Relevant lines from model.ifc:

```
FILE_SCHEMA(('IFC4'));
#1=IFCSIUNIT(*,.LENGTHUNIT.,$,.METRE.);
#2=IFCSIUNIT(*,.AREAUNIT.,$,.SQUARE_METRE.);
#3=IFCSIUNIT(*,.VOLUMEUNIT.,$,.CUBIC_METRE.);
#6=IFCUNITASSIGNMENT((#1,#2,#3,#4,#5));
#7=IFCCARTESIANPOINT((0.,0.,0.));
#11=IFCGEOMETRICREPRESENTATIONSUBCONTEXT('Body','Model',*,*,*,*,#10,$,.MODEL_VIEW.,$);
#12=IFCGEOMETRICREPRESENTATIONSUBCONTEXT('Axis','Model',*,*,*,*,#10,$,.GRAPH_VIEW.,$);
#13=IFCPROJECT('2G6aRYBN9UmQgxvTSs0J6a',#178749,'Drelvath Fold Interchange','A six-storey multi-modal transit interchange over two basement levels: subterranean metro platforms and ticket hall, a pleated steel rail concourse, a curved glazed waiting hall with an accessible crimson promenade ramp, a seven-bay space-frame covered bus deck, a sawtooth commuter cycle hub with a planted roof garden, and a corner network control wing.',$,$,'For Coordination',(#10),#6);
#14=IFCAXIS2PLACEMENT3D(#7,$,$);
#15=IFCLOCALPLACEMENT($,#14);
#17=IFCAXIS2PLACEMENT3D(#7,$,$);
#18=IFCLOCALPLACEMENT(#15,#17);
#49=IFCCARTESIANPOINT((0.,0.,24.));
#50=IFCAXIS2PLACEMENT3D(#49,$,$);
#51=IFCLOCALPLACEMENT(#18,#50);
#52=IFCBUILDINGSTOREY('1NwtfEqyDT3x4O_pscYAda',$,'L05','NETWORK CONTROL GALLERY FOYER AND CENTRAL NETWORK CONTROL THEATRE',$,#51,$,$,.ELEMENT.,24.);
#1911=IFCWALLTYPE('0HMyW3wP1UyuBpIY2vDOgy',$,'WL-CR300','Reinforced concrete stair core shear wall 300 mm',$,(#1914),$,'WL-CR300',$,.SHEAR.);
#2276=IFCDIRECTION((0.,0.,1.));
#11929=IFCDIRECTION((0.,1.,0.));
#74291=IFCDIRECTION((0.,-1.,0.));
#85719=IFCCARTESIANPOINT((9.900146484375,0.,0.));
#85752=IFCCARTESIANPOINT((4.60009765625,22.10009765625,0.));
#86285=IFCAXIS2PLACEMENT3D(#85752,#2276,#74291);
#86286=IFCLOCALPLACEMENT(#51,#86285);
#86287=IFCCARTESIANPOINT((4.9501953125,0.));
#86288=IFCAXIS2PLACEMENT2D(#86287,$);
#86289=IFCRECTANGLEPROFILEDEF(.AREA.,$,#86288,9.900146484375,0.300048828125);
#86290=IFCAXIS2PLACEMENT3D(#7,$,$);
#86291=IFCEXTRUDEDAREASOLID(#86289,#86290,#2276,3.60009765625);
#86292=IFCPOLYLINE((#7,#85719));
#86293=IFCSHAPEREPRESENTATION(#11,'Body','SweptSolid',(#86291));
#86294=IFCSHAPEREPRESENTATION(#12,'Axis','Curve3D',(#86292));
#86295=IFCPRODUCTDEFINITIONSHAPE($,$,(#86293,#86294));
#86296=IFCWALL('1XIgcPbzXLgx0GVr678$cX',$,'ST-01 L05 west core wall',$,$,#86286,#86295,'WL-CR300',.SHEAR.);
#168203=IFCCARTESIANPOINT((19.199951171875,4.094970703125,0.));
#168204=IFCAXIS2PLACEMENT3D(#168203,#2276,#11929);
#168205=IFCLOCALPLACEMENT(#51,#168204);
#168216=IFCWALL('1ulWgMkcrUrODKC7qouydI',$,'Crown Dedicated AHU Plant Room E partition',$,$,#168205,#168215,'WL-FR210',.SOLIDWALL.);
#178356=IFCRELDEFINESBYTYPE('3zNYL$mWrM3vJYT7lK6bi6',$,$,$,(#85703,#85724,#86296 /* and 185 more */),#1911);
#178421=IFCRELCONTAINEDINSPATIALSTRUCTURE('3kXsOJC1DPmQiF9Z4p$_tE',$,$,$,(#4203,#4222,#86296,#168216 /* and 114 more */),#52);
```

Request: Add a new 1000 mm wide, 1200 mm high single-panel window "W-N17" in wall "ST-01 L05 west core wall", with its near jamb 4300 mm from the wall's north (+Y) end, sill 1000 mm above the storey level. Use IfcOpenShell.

```python
import numpy as np
import ifcopenshell
import ifcopenshell.api.feature
import ifcopenshell.api.geometry
import ifcopenshell.api.root
import ifcopenshell.api.spatial
import ifcopenshell.geom
import ifcopenshell.util.element
import ifcopenshell.util.placement
import ifcopenshell.util.representation
import ifcopenshell.util.shape
import ifcopenshell.util.unit

model = ifcopenshell.open("model.ifc")
unit_scale = ifcopenshell.util.unit.calculate_unit_scale(model)
settings = ifcopenshell.geom.settings()


def volume(element):
    """Net volume in cubic metres, openings subtracted."""
    shape = ifcopenshell.geom.create_shape(settings, element)
    return ifcopenshell.util.shape.get_volume(shape.geometry)


wall = model.by_guid("1XIgcPbzXLgx0GVr678$cX")
storey = ifcopenshell.util.element.get_container(wall, ifc_class="IfcBuildingStorey")
context = ifcopenshell.util.representation.get_context(model, "Model", "Body", "MODEL_VIEW")
before = volume(wall)

width, height, from_end, sill = 1, 1.2, 4.3, 1  # metres

# The wall runs along its own X axis, and the end named is its -X end.
wall_shape = ifcopenshell.geom.create_shape(settings, wall)
x, y, z = ifcopenshell.util.shape.get_vertices(wall_shape.geometry).T
start = x.min() + from_end
face, thickness = float(y.min()), float(y.max() - y.min())
wall_matrix = ifcopenshell.util.placement.get_local_placement(wall.ObjectPlacement)
level = ifcopenshell.util.placement.get_local_placement(storey.ObjectPlacement)[2, 3]


def in_wall(x, y):
    """Placement at x, y metres in the wall's axes, at sill height."""
    matrix = wall_matrix.copy()
    matrix[:, 3] = wall_matrix @ np.array([x / unit_scale, y / unit_scale, 0.0, 1.0])
    matrix[2, 3] = level + sill / unit_scale
    return matrix


# Opening: a box that overshoots both wall faces by 50 mm.
opening = ifcopenshell.api.root.create_entity(model, ifc_class="IfcOpeningElement", predefined_type="OPENING")
box = ifcopenshell.api.geometry.add_wall_representation(
    model, context=context, length=width, height=height, thickness=thickness + 0.1
)
ifcopenshell.api.geometry.assign_representation(model, product=opening, representation=box)
ifcopenshell.api.geometry.edit_object_placement(model, product=opening, matrix=in_wall(start, face - 0.05), is_si=False)
ifcopenshell.api.feature.add_feature(model, feature=opening, element=wall)

window = ifcopenshell.api.root.create_entity(model, ifc_class="IfcWindow", name="W-N17", predefined_type="WINDOW")
window.OverallWidth, window.OverallHeight = width / unit_scale, height / unit_scale
window.PartitioningType = "SINGLE_PANEL"
body = ifcopenshell.api.geometry.add_window_representation(
    model,
    context=context,
    overall_width=window.OverallWidth,
    overall_height=window.OverallHeight,
    partition_type="SINGLE_PANEL",
)
ifcopenshell.api.geometry.assign_representation(model, product=window, representation=body)
ifcopenshell.api.spatial.assign_container(model, products=[window], relating_structure=storey)
ifcopenshell.api.feature.add_filling(model, opening=opening, element=window)

# Centre the window in the wall's thickness.
ifcopenshell.api.geometry.edit_object_placement(model, product=window, matrix=in_wall(start, face), is_si=False)
window_shape = ifcopenshell.geom.create_shape(settings, window)
depth = ifcopenshell.util.shape.get_vertices(window_shape.geometry)[:, 1]
offset = face + thickness / 2 - (depth.min() + depth.max()) / 2
ifcopenshell.api.geometry.edit_object_placement(model, product=window, matrix=in_wall(start, offset), is_si=False)

after = volume(wall)

print(f"wall volume {before:.3f} -> {after:.3f} m3")

model.write("model-out.ifc")
```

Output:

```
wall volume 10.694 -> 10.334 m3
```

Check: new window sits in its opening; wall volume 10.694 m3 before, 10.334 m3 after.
